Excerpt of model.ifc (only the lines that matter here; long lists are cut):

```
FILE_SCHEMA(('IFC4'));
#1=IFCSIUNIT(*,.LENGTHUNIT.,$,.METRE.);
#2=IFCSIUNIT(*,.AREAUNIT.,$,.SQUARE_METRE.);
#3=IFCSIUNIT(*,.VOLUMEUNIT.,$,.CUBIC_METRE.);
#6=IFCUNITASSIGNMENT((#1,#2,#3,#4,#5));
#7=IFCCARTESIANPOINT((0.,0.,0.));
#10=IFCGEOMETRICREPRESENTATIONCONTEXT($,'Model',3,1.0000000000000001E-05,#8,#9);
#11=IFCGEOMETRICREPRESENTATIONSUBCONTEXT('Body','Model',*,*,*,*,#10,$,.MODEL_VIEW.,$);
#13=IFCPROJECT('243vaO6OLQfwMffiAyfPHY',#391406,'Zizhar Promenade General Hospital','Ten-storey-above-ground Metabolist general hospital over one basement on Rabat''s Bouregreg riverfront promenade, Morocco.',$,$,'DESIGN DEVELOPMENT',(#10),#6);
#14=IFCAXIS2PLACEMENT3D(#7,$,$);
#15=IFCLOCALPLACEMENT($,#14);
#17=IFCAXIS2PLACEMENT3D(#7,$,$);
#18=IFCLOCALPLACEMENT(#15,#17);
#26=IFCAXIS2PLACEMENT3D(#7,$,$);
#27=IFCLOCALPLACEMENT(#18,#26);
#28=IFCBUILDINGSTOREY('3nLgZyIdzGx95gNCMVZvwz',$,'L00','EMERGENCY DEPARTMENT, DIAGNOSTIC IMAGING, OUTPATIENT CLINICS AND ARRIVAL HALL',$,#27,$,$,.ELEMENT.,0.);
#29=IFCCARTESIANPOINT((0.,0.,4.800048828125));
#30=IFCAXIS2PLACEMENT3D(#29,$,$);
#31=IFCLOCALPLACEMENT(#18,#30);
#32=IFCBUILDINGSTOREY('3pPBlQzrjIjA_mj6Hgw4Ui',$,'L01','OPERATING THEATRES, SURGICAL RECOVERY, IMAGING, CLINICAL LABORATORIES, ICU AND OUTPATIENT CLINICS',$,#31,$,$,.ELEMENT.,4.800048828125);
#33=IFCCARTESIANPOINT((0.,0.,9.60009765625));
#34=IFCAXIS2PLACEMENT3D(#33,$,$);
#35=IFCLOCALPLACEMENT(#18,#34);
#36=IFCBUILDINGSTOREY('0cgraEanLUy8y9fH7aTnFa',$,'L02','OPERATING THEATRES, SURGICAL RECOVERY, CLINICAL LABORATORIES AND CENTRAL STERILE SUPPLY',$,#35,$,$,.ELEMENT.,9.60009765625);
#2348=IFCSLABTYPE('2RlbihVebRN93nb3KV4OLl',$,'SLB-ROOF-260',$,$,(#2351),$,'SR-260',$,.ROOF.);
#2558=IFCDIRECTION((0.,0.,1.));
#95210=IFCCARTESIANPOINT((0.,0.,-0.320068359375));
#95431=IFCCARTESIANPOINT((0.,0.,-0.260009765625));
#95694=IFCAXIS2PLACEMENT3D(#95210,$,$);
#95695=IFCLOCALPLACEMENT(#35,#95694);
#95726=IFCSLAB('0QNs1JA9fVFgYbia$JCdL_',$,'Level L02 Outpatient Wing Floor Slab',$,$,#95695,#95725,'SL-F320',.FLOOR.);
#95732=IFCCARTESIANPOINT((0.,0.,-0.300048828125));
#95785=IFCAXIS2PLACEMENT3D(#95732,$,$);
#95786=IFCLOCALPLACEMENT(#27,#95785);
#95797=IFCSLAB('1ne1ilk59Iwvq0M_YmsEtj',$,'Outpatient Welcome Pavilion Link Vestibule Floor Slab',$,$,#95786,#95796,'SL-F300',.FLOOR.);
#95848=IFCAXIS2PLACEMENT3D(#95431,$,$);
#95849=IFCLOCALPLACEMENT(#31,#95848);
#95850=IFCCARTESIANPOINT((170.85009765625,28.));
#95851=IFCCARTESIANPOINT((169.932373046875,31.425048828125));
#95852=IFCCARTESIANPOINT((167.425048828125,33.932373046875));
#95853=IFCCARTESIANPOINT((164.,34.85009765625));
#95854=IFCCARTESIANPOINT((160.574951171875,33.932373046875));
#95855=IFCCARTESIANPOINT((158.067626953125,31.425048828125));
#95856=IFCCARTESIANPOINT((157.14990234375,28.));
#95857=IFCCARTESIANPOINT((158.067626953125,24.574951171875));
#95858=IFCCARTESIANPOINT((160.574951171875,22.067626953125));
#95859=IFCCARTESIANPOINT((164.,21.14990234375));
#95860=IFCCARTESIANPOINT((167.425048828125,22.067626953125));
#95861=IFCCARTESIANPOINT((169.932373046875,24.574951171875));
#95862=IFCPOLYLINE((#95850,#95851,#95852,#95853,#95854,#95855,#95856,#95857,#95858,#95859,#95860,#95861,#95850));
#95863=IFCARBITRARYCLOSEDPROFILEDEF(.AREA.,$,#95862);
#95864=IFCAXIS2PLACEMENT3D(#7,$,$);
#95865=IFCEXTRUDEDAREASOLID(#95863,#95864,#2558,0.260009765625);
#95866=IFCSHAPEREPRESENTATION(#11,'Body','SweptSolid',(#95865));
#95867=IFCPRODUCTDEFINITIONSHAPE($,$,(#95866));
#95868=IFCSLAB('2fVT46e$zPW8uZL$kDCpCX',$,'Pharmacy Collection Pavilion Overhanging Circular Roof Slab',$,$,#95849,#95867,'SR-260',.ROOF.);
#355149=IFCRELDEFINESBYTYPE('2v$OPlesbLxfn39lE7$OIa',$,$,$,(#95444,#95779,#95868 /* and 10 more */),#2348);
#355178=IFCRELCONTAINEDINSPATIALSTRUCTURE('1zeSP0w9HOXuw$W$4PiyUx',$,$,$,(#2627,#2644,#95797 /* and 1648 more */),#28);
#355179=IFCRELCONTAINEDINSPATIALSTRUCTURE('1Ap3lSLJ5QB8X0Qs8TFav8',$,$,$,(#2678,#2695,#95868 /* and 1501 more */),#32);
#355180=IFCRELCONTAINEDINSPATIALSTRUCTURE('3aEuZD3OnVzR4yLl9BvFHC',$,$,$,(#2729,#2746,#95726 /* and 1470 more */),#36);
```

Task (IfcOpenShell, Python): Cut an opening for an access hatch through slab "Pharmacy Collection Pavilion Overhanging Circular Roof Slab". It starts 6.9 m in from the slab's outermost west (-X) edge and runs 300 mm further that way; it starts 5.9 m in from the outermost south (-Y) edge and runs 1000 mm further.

```python
import numpy as np
import ifcopenshell
import ifcopenshell.api.feature
import ifcopenshell.api.geometry
import ifcopenshell.api.root
import ifcopenshell.geom
import ifcopenshell.util.placement
import ifcopenshell.util.representation
import ifcopenshell.util.shape
import ifcopenshell.util.unit

model = ifcopenshell.open("model.ifc")
unit_scale = ifcopenshell.util.unit.calculate_unit_scale(model)
settings = ifcopenshell.geom.settings()


def volume(element):
    """Net volume in cubic metres, openings subtracted."""
    shape = ifcopenshell.geom.create_shape(settings, element)
    return ifcopenshell.util.shape.get_volume(shape.geometry)


slab = model.by_guid("2fVT46e$zPW8uZL$kDCpCX")
before = volume(slab)

# Extent in the slab's own axes, in metres. The edges named are its -X and -Y sides.
slab_shape = ifcopenshell.geom.create_shape(settings, slab)
vertices = ifcopenshell.util.shape.get_vertices(slab_shape.geometry)
x_min, y_min, bottom = vertices.min(axis=0)
top = vertices[:, 2].max()

opening = ifcopenshell.api.root.create_entity(model, ifc_class="IfcOpeningElement", name="Access hatch opening", predefined_type="OPENING")
context = ifcopenshell.util.representation.get_context(model, "Model", "Body", "MODEL_VIEW")
width, depth = 0.3, 1
outline = [(0.0, 0.0), (width, 0.0), (width, depth), (0.0, depth), (0.0, 0.0)]
# Overshoot both faces by 50 mm so the cut is clean.
shape = ifcopenshell.api.geometry.add_slab_representation(
    model, context=context, depth=top - bottom + 0.1, polyline=outline
)
ifcopenshell.api.geometry.assign_representation(model, product=opening, representation=shape)

matrix = ifcopenshell.util.placement.get_local_placement(slab.ObjectPlacement)
matrix[:, 3] = matrix @ np.append(np.array([x_min + 6.9, y_min + 5.9, bottom - 0.05]) / unit_scale, 1.0)
ifcopenshell.api.geometry.edit_object_placement(model, product=opening, matrix=matrix, is_si=False)
ifcopenshell.api.feature.add_feature(model, feature=opening, element=slab)

after = volume(slab)

print(f"slab volume {before:.3f} -> {after:.3f} m3")

model.write("model-out.ifc")
```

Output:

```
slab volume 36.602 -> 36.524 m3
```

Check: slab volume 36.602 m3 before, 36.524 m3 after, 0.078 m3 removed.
